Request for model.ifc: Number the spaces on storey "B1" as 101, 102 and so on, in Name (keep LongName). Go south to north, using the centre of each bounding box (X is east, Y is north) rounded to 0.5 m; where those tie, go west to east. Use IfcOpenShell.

First a look at what the model holds.

```python
import ifcopenshell
import ifcopenshell.util.element
import ifcopenshell.util.placement

model = ifcopenshell.open("model.ifc")
print(model.schema)
storey = next(s for s in model.by_type("IfcBuildingStorey") if s.Name == "B1")
spaces = [e for e in ifcopenshell.util.element.get_decomposition(storey) if e.is_a("IfcSpace")]
for e in sorted(spaces, key=lambda e: e.id()):
    origin = ifcopenshell.util.placement.get_local_placement(e.ObjectPlacement)[:3, 3]
    print(e.id(), e.Name, e.LongName, origin.round(2) + 0.0, sep=" | ")
```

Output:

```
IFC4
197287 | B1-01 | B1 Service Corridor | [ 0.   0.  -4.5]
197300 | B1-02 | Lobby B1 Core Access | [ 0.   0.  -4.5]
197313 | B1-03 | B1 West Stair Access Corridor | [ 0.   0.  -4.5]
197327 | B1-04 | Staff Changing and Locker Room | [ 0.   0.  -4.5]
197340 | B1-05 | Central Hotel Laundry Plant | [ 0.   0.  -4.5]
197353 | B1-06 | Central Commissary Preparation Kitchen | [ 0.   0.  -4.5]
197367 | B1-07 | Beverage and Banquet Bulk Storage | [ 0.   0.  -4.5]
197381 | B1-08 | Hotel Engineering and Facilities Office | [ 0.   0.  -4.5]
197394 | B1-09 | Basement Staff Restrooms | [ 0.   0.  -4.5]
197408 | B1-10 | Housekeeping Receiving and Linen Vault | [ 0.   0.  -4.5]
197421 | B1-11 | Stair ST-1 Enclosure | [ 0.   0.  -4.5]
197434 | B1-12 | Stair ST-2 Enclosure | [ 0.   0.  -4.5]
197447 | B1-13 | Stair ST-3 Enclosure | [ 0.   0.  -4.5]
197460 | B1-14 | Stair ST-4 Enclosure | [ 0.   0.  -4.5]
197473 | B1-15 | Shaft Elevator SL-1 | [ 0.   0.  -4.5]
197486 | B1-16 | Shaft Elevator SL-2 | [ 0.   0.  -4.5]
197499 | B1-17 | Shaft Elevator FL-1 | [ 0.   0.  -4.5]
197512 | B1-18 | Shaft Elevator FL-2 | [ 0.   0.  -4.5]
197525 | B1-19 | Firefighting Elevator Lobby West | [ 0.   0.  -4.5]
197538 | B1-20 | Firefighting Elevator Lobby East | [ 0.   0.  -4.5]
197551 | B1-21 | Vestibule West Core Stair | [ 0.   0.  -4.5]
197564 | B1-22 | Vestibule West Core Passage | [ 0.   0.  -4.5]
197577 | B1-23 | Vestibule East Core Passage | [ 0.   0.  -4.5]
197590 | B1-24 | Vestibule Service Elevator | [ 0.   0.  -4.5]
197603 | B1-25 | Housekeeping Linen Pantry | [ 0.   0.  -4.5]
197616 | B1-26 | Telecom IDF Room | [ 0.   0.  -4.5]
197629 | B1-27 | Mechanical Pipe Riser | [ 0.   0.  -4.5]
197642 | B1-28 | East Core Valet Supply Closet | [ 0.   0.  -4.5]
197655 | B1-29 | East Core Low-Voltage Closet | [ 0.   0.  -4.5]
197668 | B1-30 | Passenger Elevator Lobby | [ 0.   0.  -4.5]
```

```python
import ifcopenshell
import ifcopenshell.geom
import ifcopenshell.util.element
import ifcopenshell.util.shape

model = ifcopenshell.open("model.ifc")
settings = ifcopenshell.geom.settings()
settings.set("use-world-coords", True)


def centre(element):
    shape = ifcopenshell.geom.create_shape(settings, element)
    return ifcopenshell.util.shape.get_bbox_centroid(shape.geometry)


storey = next(s for s in model.by_type("IfcBuildingStorey") if s.Name == "B1")
spaces = [e for e in ifcopenshell.util.element.get_decomposition(storey) if e.is_a("IfcSpace")]

# Insertion points can sit at a corner or the storey origin, so sort by the geometry (in metres).
centres = {e: centre(e) for e in spaces}
spaces.sort(key=lambda e: (round(centres[e][1] / 0.5), centres[e][0]))

for i, e in enumerate(spaces, start=1):
    number = f"1{i:02d}"
    e.Name = number
    print(e.id(), number)

model.write("model_edited.ifc")
```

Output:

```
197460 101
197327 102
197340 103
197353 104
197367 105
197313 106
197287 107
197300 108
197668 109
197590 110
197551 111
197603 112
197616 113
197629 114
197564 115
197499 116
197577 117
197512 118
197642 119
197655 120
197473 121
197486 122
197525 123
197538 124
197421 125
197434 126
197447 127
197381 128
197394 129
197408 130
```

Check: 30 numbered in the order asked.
